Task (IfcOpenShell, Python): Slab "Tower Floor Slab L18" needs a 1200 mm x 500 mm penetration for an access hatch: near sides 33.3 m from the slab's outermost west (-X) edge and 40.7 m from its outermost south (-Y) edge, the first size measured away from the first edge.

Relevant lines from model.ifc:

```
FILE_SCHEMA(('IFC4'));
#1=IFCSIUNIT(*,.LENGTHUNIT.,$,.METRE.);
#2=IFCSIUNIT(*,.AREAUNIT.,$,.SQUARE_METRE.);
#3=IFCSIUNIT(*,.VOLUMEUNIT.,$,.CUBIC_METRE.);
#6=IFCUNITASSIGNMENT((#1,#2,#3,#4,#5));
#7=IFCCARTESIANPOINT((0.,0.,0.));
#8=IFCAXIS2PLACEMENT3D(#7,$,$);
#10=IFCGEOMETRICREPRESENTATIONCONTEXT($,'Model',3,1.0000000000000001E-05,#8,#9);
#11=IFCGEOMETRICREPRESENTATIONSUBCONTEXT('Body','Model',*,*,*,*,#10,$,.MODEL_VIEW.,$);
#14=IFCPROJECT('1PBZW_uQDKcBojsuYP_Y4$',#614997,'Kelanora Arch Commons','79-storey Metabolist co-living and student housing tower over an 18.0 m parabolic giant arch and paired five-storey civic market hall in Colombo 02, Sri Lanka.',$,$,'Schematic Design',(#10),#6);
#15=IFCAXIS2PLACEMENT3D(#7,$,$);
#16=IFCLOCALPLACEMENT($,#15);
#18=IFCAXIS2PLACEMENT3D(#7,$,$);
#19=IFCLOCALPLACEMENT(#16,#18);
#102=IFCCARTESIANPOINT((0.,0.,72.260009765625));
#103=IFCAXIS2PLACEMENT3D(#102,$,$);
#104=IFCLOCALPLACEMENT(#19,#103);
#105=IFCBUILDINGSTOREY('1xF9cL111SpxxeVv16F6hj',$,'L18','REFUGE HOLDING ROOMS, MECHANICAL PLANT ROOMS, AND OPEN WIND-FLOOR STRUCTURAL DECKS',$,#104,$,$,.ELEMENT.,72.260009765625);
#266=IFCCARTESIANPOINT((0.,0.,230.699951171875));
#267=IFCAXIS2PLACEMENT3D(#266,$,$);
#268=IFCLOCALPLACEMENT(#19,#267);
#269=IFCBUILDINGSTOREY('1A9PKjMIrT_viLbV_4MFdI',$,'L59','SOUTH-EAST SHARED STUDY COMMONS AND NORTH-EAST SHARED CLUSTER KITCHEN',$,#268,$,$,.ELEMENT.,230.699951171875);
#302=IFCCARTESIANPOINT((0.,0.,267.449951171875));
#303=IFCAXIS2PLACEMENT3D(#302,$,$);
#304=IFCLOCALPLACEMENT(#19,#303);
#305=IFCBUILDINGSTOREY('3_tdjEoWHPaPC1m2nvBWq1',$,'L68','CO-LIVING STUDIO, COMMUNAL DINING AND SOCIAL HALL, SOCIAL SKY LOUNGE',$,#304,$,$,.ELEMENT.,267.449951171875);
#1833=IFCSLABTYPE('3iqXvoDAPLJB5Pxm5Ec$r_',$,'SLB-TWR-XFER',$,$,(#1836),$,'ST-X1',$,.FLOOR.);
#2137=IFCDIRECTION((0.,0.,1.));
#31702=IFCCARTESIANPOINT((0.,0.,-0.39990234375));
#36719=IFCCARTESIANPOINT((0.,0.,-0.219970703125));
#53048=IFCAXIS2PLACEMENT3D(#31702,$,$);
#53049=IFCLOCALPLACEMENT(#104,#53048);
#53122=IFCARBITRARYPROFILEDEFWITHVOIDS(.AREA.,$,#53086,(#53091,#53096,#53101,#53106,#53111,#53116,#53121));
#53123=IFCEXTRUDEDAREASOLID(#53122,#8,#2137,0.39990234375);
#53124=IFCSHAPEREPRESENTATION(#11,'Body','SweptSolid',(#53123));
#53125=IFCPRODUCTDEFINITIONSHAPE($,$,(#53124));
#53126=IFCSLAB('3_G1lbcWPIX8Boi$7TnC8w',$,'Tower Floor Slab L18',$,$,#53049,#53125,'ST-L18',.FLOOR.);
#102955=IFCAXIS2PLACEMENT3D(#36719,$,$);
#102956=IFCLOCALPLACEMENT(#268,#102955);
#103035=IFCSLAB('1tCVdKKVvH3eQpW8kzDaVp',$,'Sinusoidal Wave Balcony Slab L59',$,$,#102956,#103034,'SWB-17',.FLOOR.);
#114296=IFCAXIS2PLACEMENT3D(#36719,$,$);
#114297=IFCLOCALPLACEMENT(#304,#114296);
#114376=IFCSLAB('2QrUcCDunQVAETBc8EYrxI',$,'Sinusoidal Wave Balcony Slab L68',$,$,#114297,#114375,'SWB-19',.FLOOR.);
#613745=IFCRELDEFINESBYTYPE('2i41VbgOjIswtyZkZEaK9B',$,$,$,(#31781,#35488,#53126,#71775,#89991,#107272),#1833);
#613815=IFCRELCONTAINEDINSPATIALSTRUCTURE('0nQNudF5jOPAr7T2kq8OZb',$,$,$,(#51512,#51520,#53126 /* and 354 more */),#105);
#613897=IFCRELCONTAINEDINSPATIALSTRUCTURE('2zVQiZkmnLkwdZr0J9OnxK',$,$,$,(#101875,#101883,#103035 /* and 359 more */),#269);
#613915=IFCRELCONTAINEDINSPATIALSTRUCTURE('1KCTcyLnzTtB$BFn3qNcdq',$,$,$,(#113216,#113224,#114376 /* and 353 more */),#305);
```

```python
import numpy as np
import ifcopenshell
import ifcopenshell.api.feature
import ifcopenshell.api.geometry
import ifcopenshell.api.root
import ifcopenshell.geom
import ifcopenshell.util.placement
import ifcopenshell.util.representation
import ifcopenshell.util.shape
import ifcopenshell.util.unit

model = ifcopenshell.open("model.ifc")
unit_scale = ifcopenshell.util.unit.calculate_unit_scale(model)
settings = ifcopenshell.geom.settings()


def volume(element):
    """Net volume in cubic metres, openings subtracted."""
    shape = ifcopenshell.geom.create_shape(settings, element)
    return ifcopenshell.util.shape.get_volume(shape.geometry)


slab = model.by_guid("3_G1lbcWPIX8Boi$7TnC8w")
before = volume(slab)

# Extent in the slab's own axes, in metres. The edges named are its -X and -Y sides.
slab_shape = ifcopenshell.geom.create_shape(settings, slab)
vertices = ifcopenshell.util.shape.get_vertices(slab_shape.geometry)
x_min, y_min, bottom = vertices.min(axis=0)
top = vertices[:, 2].max()

opening = ifcopenshell.api.root.create_entity(model, ifc_class="IfcOpeningElement", name="Access hatch opening", predefined_type="OPENING")
context = ifcopenshell.util.representation.get_context(model, "Model", "Body", "MODEL_VIEW")
width, depth = 1.2, 0.5
outline = [(0.0, 0.0), (width, 0.0), (width, depth), (0.0, depth), (0.0, 0.0)]
# Overshoot both faces by 50 mm so the cut is clean.
shape = ifcopenshell.api.geometry.add_slab_representation(
    model, context=context, depth=top - bottom + 0.1, polyline=outline
)
ifcopenshell.api.geometry.assign_representation(model, product=opening, representation=shape)

matrix = ifcopenshell.util.placement.get_local_placement(slab.ObjectPlacement)
matrix[:, 3] = matrix @ np.append(np.array([x_min + 33.3, y_min + 40.7, bottom - 0.05]) / unit_scale, 1.0)
ifcopenshell.api.geometry.edit_object_placement(model, product=opening, matrix=matrix, is_si=False)
ifcopenshell.api.feature.add_feature(model, feature=opening, element=slab)

after = volume(slab)

print(f"slab volume {before:.3f} -> {after:.3f} m3")

model.write("model_updated.ifc")
```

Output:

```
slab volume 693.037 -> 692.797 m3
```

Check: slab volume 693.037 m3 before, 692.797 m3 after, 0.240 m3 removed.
